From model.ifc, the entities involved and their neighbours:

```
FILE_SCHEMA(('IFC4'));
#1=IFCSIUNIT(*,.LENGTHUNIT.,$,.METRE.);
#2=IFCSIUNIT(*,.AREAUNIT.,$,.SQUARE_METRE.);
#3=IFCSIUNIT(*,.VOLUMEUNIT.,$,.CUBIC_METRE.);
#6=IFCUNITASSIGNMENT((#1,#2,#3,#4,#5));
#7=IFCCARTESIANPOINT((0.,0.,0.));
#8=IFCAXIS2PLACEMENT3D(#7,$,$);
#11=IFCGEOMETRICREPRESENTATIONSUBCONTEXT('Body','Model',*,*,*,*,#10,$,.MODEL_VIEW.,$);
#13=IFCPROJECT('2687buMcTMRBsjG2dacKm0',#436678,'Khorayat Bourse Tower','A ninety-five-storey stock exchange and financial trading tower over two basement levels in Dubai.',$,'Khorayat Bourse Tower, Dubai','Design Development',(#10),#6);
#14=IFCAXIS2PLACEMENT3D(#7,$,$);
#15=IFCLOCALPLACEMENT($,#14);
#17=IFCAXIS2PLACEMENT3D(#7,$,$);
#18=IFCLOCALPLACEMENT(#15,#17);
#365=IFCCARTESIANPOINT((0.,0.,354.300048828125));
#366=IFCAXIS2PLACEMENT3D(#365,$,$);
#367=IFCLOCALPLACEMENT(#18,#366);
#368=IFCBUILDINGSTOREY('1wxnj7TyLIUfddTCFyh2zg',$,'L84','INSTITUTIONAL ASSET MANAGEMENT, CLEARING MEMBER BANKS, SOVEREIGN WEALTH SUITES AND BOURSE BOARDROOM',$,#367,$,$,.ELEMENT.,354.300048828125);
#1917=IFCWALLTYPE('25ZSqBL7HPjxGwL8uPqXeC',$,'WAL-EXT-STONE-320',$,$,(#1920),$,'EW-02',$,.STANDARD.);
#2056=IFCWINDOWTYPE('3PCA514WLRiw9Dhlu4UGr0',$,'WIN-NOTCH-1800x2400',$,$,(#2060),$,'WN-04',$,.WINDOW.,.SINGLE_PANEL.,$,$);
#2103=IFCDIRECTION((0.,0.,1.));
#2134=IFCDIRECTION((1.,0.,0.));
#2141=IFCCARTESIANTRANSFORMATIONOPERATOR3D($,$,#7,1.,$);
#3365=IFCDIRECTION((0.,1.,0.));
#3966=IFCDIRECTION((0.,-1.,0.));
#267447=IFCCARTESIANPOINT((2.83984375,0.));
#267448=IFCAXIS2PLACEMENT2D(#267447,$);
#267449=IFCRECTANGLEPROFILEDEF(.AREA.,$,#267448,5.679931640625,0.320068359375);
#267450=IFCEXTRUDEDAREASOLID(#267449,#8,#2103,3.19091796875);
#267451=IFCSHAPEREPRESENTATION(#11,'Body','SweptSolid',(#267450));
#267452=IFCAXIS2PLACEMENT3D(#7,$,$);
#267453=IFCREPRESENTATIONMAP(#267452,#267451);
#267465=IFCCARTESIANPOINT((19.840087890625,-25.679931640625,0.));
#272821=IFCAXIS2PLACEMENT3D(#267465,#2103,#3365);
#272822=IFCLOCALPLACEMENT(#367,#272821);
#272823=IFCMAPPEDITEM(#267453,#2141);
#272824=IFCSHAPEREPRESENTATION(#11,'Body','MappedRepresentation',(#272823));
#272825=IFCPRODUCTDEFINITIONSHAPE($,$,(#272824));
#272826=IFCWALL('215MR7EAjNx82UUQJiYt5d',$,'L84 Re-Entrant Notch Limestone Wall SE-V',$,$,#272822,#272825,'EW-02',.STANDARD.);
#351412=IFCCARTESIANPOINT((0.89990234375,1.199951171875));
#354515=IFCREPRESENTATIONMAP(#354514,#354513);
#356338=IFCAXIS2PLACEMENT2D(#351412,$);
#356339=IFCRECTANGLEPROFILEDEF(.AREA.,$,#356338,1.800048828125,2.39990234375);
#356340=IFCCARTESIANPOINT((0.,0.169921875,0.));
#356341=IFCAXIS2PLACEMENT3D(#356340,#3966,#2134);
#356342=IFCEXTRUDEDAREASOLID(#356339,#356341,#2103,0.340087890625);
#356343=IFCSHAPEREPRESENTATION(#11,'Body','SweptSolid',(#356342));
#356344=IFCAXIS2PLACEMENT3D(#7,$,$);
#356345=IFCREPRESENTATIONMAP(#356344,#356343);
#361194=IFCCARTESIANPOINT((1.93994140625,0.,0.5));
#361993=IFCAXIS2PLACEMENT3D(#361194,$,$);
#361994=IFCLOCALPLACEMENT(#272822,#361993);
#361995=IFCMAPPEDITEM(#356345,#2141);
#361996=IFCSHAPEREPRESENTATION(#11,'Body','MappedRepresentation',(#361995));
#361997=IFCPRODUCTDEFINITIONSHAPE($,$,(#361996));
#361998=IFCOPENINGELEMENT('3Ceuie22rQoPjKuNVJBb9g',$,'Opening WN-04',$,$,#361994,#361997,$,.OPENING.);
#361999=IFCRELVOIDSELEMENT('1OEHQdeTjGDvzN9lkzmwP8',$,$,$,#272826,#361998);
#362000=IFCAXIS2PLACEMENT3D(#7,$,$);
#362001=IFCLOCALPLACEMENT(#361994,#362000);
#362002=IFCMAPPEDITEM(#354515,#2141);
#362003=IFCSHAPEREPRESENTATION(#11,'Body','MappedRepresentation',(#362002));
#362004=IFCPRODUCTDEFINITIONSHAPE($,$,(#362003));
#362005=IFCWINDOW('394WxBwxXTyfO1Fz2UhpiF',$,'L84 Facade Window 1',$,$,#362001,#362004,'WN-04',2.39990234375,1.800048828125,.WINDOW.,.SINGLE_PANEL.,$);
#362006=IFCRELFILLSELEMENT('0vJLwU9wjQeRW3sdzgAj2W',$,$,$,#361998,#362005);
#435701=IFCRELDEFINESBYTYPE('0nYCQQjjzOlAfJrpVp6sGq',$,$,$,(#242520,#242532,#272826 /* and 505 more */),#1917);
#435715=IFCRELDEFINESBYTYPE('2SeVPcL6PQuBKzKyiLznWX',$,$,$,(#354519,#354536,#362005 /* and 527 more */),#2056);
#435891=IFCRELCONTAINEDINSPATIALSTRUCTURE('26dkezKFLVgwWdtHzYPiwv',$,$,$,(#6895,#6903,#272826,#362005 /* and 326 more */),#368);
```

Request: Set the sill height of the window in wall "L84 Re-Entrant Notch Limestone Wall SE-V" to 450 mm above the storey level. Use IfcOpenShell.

```python
import numpy as np
import ifcopenshell
import ifcopenshell.api.geometry
import ifcopenshell.geom
import ifcopenshell.util.element
import ifcopenshell.util.placement
import ifcopenshell.util.shape
import ifcopenshell.util.unit

model = ifcopenshell.open("model.ifc")
unit_scale = ifcopenshell.util.unit.calculate_unit_scale(model)

window = model.by_id(362005)
opening = window.FillsVoids[0].RelatingOpeningElement
storey = ifcopenshell.util.element.get_container(window, ifc_class="IfcBuildingStorey")
level = ifcopenshell.util.placement.get_local_placement(storey.ObjectPlacement)[2, 3]

# The opening's origin need not be at the sill, so measure its lowest point.
shape = ifcopenshell.geom.create_shape(ifcopenshell.geom.settings(), opening)
bottom = ifcopenshell.util.shape.get_shape_bottom_elevation(shape, shape.geometry) / unit_scale
dz = level + 0.45 - bottom

shift = np.array([0.0, 0.0, dz])
# The window is placed relative to its opening, so it follows when the opening moves.
matrix = ifcopenshell.util.placement.get_local_placement(opening.ObjectPlacement)
matrix[:3, 3] += shift
ifcopenshell.api.geometry.edit_object_placement(
    model, product=opening, matrix=matrix, is_si=False, should_transform_children=True
)

print(f"moved by {dz * unit_scale:+.3f} m")

model.write("model_rev.ifc")
```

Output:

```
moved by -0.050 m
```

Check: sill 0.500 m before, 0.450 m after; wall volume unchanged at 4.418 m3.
